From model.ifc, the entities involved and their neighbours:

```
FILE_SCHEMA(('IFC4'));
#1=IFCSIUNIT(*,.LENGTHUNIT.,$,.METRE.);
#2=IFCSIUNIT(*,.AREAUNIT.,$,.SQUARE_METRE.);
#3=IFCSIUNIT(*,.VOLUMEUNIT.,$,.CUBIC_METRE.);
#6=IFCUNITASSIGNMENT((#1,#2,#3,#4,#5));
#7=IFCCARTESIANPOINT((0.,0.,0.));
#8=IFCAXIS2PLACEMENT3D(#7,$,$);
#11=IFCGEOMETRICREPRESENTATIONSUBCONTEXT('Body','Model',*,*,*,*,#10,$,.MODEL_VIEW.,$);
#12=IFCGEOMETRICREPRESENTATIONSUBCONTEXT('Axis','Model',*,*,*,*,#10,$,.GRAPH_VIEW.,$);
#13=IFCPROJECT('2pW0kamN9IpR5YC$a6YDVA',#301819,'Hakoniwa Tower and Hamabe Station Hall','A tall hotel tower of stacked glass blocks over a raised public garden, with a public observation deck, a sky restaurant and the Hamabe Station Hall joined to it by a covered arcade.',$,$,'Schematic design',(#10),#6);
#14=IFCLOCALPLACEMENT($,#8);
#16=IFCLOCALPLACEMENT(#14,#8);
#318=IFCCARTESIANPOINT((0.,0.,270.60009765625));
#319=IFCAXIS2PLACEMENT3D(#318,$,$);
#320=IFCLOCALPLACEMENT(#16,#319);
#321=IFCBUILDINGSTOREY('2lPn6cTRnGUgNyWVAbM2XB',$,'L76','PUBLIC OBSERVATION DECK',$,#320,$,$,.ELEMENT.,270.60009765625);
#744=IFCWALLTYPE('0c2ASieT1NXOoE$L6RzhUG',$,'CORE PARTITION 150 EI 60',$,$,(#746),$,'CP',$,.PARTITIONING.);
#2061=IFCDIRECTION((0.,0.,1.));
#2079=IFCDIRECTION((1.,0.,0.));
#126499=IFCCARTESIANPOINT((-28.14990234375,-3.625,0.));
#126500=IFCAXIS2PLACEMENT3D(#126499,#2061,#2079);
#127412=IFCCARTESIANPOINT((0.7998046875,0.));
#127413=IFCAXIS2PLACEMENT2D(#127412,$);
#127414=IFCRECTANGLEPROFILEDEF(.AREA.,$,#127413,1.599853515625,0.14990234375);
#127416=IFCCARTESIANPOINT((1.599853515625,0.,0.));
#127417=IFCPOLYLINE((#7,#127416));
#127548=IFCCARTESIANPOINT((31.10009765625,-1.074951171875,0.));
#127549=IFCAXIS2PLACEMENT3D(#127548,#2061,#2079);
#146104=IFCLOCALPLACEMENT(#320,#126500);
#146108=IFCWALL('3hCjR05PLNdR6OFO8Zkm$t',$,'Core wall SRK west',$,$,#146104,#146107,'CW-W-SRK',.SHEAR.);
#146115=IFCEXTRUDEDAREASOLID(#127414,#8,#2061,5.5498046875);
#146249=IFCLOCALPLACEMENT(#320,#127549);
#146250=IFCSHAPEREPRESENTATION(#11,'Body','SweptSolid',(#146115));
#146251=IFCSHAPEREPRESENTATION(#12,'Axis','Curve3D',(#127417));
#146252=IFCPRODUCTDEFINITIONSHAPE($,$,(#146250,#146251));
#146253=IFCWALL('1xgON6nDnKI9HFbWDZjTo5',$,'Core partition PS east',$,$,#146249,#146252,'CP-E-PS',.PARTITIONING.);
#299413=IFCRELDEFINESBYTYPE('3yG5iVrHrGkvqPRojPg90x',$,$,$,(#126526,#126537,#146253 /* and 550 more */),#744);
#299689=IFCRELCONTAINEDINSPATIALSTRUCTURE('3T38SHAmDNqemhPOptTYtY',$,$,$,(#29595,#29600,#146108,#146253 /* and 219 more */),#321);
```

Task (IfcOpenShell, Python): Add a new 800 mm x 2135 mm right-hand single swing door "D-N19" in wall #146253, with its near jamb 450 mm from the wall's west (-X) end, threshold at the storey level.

```python
import numpy as np
import ifcopenshell
import ifcopenshell.api.feature
import ifcopenshell.api.geometry
import ifcopenshell.api.root
import ifcopenshell.api.spatial
import ifcopenshell.geom
import ifcopenshell.util.element
import ifcopenshell.util.placement
import ifcopenshell.util.representation
import ifcopenshell.util.shape
import ifcopenshell.util.unit

model = ifcopenshell.open("model.ifc")
unit_scale = ifcopenshell.util.unit.calculate_unit_scale(model)
settings = ifcopenshell.geom.settings()


def volume(element):
    """Net volume in cubic metres, openings subtracted."""
    shape = ifcopenshell.geom.create_shape(settings, element)
    return ifcopenshell.util.shape.get_volume(shape.geometry)


wall = model.by_id(146253)
storey = ifcopenshell.util.element.get_container(wall, ifc_class="IfcBuildingStorey")
context = ifcopenshell.util.representation.get_context(model, "Model", "Body", "MODEL_VIEW")
before = volume(wall)

width, height, from_end, sill = 0.8, 2.135, 0.45, 0.0  # metres

# The wall runs along its own X axis, and the end named is its -X end.
wall_shape = ifcopenshell.geom.create_shape(settings, wall)
x, y, z = ifcopenshell.util.shape.get_vertices(wall_shape.geometry).T
start = x.min() + from_end
face, thickness = float(y.min()), float(y.max() - y.min())
wall_matrix = ifcopenshell.util.placement.get_local_placement(wall.ObjectPlacement)
level = ifcopenshell.util.placement.get_local_placement(storey.ObjectPlacement)[2, 3]


def in_wall(x, y):
    """Placement at x, y metres in the wall's axes, at sill height."""
    matrix = wall_matrix.copy()
    matrix[:, 3] = wall_matrix @ np.array([x / unit_scale, y / unit_scale, 0.0, 1.0])
    matrix[2, 3] = level + sill / unit_scale
    return matrix


# Opening: a box that overshoots both wall faces by 50 mm.
opening = ifcopenshell.api.root.create_entity(model, ifc_class="IfcOpeningElement", predefined_type="OPENING")
box = ifcopenshell.api.geometry.add_wall_representation(
    model, context=context, length=width, height=height, thickness=thickness + 0.1
)
ifcopenshell.api.geometry.assign_representation(model, product=opening, representation=box)
ifcopenshell.api.geometry.edit_object_placement(model, product=opening, matrix=in_wall(start, face - 0.05), is_si=False)
ifcopenshell.api.feature.add_feature(model, feature=opening, element=wall)

door = ifcopenshell.api.root.create_entity(model, ifc_class="IfcDoor", name="D-N19", predefined_type="DOOR")
door.OverallWidth, door.OverallHeight = width / unit_scale, height / unit_scale
door.OperationType = "SINGLE_SWING_RIGHT"
body = ifcopenshell.api.geometry.add_door_representation(
    model,
    context=context,
    overall_width=door.OverallWidth,
    overall_height=door.OverallHeight,
    operation_type="SINGLE_SWING_RIGHT",
    lining_properties={"LiningDepth": thickness / unit_scale, "ThresholdDepth": thickness / unit_scale},
)
ifcopenshell.api.geometry.assign_representation(model, product=door, representation=body)
ifcopenshell.api.spatial.assign_container(model, products=[door], relating_structure=storey)
ifcopenshell.api.feature.add_filling(model, opening=opening, element=door)

# The lining spans the wall, so the door starts at the wall face.
ifcopenshell.api.geometry.edit_object_placement(model, product=door, matrix=in_wall(start, face), is_si=False)

after = volume(wall)

print(f"wall volume {before:.3f} -> {after:.3f} m3")

model.write("model-out.ifc")
```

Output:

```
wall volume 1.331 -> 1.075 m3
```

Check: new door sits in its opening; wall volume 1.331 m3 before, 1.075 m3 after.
